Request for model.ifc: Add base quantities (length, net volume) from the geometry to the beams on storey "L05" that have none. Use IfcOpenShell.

First a look at what the model holds.

```python
import ifcopenshell
import ifcopenshell.util.element
import ifcopenshell.util.unit

model = ifcopenshell.open("model.ifc")
print(model.schema)
for unit_type in ("LENGTHUNIT", "AREAUNIT", "VOLUMEUNIT"):
    print(unit_type, ifcopenshell.util.unit.calculate_unit_scale(model, unit_type))
storey = next(s for s in model.by_type("IfcBuildingStorey") if s.Name == "L05")
beams = [e for e in ifcopenshell.util.element.get_decomposition(storey) if e.is_a("IfcBeam")]
for e in sorted(beams, key=lambda e: e.id()):
    print(e.id(), e.is_a(), e.Name, list(ifcopenshell.util.element.get_psets(e, qtos_only=True)), sep=" | ")
```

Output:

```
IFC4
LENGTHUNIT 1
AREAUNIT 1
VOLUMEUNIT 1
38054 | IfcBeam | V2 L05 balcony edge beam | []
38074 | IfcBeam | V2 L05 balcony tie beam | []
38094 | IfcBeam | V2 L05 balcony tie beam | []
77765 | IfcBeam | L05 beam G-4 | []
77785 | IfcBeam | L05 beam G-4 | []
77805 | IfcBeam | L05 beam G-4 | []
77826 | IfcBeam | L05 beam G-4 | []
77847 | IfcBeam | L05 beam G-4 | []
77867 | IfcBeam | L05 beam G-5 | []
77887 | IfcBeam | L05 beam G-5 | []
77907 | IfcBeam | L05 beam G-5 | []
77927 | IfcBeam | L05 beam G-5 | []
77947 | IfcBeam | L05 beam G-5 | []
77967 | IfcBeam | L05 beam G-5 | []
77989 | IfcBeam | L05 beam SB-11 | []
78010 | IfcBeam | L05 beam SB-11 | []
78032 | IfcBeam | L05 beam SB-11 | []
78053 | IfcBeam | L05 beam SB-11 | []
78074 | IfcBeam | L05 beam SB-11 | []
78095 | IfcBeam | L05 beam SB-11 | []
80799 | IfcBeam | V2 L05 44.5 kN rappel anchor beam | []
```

```python
import ifcopenshell
import ifcopenshell.api.pset
import ifcopenshell.geom
import ifcopenshell.util.element
import ifcopenshell.util.shape
import ifcopenshell.util.unit

model = ifcopenshell.open("model.ifc")
unit_scale = ifcopenshell.util.unit.calculate_unit_scale(model)
volume_scale = ifcopenshell.util.unit.calculate_unit_scale(model, "VOLUMEUNIT")
settings = ifcopenshell.geom.settings()

storey = next(s for s in model.by_type("IfcBuildingStorey") if s.Name == "L05")
beams = [e for e in ifcopenshell.util.element.get_decomposition(storey) if e.is_a("IfcBeam")]

for e in sorted(beams, key=lambda e: e.id()):
    if ifcopenshell.util.element.get_psets(e, qtos_only=True, should_inherit=False):
        continue
    # Geometry comes back in metres, in the element's own axes.
    shape = ifcopenshell.geom.create_shape(settings, e)
    values = {
        "Length": ifcopenshell.util.shape.get_max_xyz(shape.geometry) / unit_scale,
        "NetVolume": ifcopenshell.util.shape.get_volume(shape.geometry) / volume_scale,
    }
    qto = ifcopenshell.api.pset.add_qto(model, product=e, name="Qto_BeamBaseQuantities")
    ifcopenshell.api.pset.edit_qto(model, qto=qto, properties=values)
    print(e.id(), {k: round(v, 3) for k, v in values.items()})

model.write("model_updated.ifc")
```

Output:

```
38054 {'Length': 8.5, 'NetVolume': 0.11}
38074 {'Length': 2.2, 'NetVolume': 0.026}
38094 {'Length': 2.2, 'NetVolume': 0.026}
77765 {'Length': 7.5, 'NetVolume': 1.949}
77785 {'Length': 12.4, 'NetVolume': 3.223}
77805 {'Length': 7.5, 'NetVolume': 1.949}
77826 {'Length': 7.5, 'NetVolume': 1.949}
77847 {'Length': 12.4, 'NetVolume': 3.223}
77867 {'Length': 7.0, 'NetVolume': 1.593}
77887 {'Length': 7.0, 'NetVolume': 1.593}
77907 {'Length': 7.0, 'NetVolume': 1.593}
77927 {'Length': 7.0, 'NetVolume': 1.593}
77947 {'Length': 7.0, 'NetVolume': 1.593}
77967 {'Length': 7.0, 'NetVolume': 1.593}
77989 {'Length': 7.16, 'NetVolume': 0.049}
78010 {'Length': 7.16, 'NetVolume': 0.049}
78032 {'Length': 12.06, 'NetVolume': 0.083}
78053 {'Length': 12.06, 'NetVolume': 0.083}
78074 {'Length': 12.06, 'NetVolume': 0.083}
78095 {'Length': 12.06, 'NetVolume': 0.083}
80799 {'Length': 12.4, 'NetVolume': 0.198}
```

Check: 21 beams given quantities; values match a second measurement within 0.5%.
